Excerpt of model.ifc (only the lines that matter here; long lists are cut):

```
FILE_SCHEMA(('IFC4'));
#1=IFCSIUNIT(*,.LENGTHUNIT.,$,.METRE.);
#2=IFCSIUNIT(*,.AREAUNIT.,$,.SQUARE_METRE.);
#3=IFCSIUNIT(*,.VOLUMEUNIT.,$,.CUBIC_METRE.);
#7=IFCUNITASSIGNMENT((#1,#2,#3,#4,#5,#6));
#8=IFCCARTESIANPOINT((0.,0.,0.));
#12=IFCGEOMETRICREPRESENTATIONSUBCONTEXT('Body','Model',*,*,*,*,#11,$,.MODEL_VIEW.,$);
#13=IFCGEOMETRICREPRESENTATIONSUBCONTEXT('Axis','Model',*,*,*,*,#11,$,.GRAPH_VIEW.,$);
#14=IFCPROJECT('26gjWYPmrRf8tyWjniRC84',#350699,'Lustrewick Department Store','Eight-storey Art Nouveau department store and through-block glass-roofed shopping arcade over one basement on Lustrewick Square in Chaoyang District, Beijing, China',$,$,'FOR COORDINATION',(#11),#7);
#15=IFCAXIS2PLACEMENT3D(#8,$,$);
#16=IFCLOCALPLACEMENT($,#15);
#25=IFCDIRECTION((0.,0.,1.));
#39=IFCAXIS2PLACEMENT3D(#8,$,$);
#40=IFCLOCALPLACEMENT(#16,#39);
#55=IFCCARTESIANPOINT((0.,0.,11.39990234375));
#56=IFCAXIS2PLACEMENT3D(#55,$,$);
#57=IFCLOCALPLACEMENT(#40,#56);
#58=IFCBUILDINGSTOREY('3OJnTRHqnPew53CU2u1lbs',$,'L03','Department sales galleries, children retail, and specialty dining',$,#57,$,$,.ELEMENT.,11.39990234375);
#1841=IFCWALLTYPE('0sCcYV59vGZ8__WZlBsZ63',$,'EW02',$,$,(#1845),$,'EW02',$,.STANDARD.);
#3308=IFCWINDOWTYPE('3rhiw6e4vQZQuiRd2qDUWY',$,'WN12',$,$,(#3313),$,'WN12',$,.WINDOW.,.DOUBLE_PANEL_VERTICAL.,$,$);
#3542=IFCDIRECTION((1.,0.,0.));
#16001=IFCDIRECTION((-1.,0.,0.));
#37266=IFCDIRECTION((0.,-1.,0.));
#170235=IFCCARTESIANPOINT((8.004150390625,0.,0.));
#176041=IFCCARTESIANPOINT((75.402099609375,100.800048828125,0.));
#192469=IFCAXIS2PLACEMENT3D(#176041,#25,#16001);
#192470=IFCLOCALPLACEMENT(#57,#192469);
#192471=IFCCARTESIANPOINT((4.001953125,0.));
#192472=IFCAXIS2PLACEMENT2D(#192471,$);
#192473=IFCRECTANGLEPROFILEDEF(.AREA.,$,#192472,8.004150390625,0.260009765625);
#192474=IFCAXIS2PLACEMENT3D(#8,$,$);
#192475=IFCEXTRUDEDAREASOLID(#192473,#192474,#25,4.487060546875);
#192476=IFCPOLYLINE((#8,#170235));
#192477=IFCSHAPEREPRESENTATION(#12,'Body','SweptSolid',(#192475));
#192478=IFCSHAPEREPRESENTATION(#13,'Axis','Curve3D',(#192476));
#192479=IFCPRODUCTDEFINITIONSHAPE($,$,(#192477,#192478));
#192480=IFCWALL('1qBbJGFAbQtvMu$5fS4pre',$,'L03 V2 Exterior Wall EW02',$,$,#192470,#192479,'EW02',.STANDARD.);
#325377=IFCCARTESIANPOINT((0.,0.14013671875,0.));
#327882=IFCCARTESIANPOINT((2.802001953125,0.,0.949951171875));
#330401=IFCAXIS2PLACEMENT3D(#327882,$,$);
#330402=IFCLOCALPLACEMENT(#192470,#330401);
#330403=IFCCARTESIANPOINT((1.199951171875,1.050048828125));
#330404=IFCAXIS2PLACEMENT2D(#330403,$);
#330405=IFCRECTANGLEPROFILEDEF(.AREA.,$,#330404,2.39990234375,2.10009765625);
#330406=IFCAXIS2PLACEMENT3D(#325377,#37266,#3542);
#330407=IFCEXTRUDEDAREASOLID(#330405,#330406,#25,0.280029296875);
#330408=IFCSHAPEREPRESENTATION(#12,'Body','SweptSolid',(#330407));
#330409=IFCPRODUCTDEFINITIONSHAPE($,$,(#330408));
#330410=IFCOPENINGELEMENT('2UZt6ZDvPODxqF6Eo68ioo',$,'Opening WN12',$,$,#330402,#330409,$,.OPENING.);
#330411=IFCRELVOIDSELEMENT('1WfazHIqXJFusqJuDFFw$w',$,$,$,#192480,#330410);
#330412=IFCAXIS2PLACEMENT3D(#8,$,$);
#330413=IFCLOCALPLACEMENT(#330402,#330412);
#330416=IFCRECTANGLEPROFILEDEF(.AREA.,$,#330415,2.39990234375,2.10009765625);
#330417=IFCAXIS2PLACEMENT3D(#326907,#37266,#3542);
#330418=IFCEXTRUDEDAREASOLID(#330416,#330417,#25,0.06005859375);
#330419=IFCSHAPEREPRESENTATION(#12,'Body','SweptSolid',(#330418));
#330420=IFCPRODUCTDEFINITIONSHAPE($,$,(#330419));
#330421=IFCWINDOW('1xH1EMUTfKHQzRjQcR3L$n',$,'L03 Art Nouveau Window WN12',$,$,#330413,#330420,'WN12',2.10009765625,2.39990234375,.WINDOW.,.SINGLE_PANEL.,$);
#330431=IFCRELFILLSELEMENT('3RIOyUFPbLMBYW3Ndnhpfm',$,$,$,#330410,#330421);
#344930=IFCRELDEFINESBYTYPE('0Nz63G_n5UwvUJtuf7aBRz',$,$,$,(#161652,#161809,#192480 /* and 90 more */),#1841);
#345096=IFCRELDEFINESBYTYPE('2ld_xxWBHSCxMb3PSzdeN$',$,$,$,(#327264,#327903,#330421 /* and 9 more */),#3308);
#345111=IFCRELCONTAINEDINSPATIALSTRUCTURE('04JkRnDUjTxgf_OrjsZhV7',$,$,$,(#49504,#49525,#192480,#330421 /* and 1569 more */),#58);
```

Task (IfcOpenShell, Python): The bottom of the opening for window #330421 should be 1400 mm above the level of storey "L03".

```python
import numpy as np
import ifcopenshell
import ifcopenshell.api.geometry
import ifcopenshell.geom
import ifcopenshell.util.element
import ifcopenshell.util.placement
import ifcopenshell.util.shape
import ifcopenshell.util.unit

model = ifcopenshell.open("model.ifc")
unit_scale = ifcopenshell.util.unit.calculate_unit_scale(model)

window = model.by_guid("1xH1EMUTfKHQzRjQcR3L$n")
opening = window.FillsVoids[0].RelatingOpeningElement
storey = ifcopenshell.util.element.get_container(window, ifc_class="IfcBuildingStorey")
level = ifcopenshell.util.placement.get_local_placement(storey.ObjectPlacement)[2, 3]

# The opening's origin need not be at the sill, so measure its lowest point.
shape = ifcopenshell.geom.create_shape(ifcopenshell.geom.settings(), opening)
bottom = ifcopenshell.util.shape.get_shape_bottom_elevation(shape, shape.geometry) / unit_scale
dz = level + 1.4 - bottom

shift = np.array([0.0, 0.0, dz])
# The window is placed relative to its opening, so it follows when the opening moves.
matrix = ifcopenshell.util.placement.get_local_placement(opening.ObjectPlacement)
matrix[:3, 3] += shift
ifcopenshell.api.geometry.edit_object_placement(
    model, product=opening, matrix=matrix, is_si=False, should_transform_children=True
)

print(f"moved by {dz * unit_scale:+.3f} m")

model.write("model-out.ifc")
```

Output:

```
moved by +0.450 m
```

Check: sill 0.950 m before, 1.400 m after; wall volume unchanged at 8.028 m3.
